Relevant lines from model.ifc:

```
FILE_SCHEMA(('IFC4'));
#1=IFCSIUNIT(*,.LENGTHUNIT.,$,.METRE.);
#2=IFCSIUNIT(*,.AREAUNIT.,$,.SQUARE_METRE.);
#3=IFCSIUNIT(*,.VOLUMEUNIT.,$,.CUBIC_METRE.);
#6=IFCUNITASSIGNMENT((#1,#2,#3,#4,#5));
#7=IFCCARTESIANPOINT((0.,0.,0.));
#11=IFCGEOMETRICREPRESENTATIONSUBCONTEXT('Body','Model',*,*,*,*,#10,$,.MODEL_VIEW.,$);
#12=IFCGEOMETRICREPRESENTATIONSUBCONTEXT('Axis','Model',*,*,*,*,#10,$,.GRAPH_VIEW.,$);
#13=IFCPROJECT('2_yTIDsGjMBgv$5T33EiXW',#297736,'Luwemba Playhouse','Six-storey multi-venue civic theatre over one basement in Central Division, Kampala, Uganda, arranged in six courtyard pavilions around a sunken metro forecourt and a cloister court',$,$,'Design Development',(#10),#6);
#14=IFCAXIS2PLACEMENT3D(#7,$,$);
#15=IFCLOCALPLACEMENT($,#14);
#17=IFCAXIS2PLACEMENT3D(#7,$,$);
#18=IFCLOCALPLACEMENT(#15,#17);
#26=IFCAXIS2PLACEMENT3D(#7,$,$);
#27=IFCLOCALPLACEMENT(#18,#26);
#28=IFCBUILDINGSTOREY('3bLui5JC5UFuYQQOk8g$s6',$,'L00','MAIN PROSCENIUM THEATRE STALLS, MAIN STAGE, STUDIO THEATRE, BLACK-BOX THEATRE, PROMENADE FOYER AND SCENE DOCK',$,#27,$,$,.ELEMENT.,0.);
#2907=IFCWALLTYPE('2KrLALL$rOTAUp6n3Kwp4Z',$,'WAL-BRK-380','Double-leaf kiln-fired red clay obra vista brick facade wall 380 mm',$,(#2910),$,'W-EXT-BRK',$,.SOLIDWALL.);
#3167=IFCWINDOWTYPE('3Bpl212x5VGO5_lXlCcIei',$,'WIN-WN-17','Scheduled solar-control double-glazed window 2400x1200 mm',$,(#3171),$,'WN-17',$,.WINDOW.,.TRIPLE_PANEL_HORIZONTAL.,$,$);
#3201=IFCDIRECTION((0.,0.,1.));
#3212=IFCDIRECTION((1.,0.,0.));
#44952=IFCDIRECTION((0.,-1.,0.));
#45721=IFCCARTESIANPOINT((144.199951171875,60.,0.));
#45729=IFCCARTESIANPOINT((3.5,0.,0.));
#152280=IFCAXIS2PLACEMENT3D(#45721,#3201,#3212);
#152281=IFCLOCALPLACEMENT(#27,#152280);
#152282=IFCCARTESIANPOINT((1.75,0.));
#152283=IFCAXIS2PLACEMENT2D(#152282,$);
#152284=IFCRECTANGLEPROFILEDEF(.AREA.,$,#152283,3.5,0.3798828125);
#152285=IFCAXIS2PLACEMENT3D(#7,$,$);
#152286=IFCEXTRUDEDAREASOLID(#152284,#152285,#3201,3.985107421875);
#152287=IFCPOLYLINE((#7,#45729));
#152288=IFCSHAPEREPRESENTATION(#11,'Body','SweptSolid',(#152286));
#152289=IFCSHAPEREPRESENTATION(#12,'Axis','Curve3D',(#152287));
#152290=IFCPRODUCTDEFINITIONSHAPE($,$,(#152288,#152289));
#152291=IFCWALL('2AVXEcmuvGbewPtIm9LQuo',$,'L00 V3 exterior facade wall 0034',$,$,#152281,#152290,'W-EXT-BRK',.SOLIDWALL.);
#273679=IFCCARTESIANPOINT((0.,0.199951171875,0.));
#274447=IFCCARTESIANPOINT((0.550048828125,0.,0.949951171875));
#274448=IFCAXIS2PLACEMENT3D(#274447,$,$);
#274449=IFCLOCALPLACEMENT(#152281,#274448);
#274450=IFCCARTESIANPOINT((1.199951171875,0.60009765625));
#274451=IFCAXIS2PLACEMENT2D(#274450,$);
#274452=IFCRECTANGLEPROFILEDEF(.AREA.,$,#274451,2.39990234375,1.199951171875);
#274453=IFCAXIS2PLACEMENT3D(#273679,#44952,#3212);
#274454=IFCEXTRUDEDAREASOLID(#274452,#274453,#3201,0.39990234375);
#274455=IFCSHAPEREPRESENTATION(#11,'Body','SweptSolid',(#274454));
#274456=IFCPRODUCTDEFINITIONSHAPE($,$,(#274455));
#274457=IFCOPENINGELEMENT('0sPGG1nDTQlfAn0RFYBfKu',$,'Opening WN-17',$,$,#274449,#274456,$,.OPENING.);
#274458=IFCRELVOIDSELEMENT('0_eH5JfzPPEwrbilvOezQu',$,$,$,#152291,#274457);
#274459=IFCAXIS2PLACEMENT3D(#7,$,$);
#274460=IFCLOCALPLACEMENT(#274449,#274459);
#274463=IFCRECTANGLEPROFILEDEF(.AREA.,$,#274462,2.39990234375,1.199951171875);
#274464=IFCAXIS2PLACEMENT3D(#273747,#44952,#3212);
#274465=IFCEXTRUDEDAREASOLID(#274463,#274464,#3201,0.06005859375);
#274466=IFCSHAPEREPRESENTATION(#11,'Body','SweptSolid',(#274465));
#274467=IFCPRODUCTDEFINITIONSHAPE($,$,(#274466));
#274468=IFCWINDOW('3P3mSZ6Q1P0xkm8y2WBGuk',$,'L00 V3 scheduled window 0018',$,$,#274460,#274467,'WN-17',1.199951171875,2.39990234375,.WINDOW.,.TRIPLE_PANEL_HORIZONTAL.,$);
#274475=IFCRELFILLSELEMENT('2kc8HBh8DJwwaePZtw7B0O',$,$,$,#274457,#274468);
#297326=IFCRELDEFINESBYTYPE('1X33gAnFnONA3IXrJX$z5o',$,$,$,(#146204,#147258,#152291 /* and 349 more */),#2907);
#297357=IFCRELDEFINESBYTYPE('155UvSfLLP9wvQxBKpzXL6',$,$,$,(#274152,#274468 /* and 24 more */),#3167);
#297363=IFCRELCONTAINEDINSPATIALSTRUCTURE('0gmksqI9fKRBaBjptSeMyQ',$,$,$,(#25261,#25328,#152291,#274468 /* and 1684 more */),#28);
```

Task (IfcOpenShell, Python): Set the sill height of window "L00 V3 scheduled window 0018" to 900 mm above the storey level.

```python
import numpy as np
import ifcopenshell
import ifcopenshell.api.geometry
import ifcopenshell.geom
import ifcopenshell.util.element
import ifcopenshell.util.placement
import ifcopenshell.util.shape
import ifcopenshell.util.unit

model = ifcopenshell.open("model.ifc")
unit_scale = ifcopenshell.util.unit.calculate_unit_scale(model)

window = model.by_guid("3P3mSZ6Q1P0xkm8y2WBGuk")
opening = window.FillsVoids[0].RelatingOpeningElement
storey = ifcopenshell.util.element.get_container(window, ifc_class="IfcBuildingStorey")
level = ifcopenshell.util.placement.get_local_placement(storey.ObjectPlacement)[2, 3]

# The opening's origin need not be at the sill, so measure its lowest point.
shape = ifcopenshell.geom.create_shape(ifcopenshell.geom.settings(), opening)
bottom = ifcopenshell.util.shape.get_shape_bottom_elevation(shape, shape.geometry) / unit_scale
dz = level + 0.9 / unit_scale - bottom

shift = np.array([0.0, 0.0, dz])
# The window is placed relative to its opening, so it follows when the opening moves.
matrix = ifcopenshell.util.placement.get_local_placement(opening.ObjectPlacement)
matrix[:3, 3] += shift
ifcopenshell.api.geometry.edit_object_placement(
    model, product=opening, matrix=matrix, is_si=False, should_transform_children=True
)

print(f"moved by {dz * unit_scale:+.3f} m")

model.write("model_v2.ifc")
```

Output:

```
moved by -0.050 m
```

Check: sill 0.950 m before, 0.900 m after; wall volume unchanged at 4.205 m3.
